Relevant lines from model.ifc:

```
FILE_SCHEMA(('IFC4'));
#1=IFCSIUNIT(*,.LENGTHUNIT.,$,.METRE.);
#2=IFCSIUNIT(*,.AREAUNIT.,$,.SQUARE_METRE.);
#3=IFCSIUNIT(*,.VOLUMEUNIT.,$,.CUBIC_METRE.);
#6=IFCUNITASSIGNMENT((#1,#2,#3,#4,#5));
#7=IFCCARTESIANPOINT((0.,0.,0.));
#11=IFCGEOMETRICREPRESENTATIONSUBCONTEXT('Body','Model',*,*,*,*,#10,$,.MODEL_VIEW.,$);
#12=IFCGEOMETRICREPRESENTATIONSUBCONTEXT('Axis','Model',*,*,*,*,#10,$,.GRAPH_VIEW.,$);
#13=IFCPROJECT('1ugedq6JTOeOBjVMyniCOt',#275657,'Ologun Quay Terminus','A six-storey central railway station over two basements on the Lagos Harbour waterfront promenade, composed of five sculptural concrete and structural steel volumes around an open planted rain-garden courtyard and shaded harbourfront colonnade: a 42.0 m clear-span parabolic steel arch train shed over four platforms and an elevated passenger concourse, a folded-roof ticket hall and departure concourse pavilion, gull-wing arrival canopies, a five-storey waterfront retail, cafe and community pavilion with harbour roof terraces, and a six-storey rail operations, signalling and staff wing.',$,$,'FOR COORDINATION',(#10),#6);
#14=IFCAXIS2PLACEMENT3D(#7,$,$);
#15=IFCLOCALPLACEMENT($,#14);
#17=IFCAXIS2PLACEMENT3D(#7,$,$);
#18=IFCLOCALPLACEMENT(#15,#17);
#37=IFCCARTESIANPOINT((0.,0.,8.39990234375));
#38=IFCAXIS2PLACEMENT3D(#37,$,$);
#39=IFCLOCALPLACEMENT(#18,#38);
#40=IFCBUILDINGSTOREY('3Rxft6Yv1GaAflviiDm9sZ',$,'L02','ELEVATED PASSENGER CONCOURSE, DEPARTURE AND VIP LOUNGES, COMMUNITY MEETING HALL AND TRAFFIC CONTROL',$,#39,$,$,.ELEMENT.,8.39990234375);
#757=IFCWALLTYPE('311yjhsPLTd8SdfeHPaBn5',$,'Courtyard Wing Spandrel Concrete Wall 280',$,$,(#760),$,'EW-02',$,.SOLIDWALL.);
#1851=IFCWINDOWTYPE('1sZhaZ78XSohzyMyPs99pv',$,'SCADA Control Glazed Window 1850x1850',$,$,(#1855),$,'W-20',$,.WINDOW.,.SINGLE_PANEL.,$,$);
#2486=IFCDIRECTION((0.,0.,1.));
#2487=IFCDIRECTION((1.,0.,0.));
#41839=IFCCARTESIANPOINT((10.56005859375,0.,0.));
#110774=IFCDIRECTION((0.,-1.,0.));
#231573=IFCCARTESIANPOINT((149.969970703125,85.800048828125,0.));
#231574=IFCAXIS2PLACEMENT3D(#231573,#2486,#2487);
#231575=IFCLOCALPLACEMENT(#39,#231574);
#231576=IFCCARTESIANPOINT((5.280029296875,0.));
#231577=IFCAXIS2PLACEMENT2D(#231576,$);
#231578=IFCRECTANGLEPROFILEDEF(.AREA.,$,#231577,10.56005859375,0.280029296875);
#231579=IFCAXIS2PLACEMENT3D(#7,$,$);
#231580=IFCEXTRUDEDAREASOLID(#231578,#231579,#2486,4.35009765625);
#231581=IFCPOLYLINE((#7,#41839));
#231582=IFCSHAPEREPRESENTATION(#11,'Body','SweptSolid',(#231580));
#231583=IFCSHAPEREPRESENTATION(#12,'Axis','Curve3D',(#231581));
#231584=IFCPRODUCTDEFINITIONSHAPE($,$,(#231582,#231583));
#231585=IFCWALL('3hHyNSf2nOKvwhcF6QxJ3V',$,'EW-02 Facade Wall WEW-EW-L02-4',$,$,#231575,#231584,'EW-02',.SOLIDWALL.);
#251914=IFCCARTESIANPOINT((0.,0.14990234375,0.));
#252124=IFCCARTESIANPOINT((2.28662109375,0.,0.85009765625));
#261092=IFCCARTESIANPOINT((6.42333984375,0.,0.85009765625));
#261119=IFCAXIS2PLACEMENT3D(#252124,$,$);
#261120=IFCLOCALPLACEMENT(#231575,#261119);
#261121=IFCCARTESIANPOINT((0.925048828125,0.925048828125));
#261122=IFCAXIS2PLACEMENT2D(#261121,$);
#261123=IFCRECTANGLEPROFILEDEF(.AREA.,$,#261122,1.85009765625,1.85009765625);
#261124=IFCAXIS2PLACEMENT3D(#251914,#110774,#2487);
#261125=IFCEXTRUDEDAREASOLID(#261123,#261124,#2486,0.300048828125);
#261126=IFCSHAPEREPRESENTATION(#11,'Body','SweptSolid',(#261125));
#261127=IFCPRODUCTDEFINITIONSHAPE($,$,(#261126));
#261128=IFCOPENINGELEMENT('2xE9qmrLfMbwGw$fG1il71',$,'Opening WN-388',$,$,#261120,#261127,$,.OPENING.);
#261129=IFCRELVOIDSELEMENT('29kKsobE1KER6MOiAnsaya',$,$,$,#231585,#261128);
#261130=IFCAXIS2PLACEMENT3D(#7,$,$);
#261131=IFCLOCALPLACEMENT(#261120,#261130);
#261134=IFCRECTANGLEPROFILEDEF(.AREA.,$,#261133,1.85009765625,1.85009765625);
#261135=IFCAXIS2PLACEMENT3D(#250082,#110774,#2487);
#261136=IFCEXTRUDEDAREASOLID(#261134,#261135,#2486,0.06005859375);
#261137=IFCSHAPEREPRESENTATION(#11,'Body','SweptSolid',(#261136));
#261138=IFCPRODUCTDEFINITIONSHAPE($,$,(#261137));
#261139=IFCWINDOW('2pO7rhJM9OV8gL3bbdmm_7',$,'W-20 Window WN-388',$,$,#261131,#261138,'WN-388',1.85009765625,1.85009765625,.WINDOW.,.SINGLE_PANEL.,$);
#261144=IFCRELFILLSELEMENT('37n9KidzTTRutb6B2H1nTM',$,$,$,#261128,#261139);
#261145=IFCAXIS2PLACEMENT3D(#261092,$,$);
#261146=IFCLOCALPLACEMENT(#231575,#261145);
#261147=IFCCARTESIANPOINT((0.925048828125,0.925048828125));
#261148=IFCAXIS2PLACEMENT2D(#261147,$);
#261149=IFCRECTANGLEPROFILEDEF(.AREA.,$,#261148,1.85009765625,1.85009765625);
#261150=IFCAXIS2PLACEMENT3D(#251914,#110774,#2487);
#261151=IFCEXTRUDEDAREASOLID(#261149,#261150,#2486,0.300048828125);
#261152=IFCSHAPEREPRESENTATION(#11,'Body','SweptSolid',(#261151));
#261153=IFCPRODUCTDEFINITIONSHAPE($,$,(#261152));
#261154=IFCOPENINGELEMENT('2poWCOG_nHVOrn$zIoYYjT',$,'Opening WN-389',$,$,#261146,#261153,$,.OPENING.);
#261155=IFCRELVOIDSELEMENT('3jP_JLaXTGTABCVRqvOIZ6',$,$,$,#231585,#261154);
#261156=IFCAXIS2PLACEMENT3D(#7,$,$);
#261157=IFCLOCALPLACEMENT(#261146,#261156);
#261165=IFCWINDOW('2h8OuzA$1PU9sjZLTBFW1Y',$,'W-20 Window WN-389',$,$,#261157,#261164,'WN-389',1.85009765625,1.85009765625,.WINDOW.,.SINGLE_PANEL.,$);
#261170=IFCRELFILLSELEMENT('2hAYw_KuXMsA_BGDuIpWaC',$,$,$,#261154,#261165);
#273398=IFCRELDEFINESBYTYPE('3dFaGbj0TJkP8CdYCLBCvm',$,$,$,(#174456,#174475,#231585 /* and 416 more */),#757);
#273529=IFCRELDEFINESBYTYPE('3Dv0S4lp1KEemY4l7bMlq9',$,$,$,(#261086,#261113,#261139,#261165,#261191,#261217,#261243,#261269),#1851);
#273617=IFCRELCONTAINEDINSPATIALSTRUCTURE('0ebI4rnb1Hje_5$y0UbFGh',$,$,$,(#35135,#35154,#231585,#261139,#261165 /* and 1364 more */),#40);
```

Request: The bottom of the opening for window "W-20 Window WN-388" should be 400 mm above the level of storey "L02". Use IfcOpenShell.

```python
import numpy as np
import ifcopenshell
import ifcopenshell.api.geometry
import ifcopenshell.geom
import ifcopenshell.util.element
import ifcopenshell.util.placement
import ifcopenshell.util.shape
import ifcopenshell.util.unit

model = ifcopenshell.open("model.ifc")
unit_scale = ifcopenshell.util.unit.calculate_unit_scale(model)

window = model.by_guid("2pO7rhJM9OV8gL3bbdmm_7")
opening = window.FillsVoids[0].RelatingOpeningElement
storey = ifcopenshell.util.element.get_container(window, ifc_class="IfcBuildingStorey")
level = ifcopenshell.util.placement.get_local_placement(storey.ObjectPlacement)[2, 3]

# The opening's origin need not be at the sill, so measure its lowest point.
shape = ifcopenshell.geom.create_shape(ifcopenshell.geom.settings(), opening)
bottom = ifcopenshell.util.shape.get_shape_bottom_elevation(shape, shape.geometry) / unit_scale
dz = level + 0.4 - bottom

shift = np.array([0.0, 0.0, dz])
# The window is placed relative to its opening, so it follows when the opening moves.
matrix = ifcopenshell.util.placement.get_local_placement(opening.ObjectPlacement)
matrix[:3, 3] += shift
ifcopenshell.api.geometry.edit_object_placement(
    model, product=opening, matrix=matrix, is_si=False, should_transform_children=True
)

print(f"moved by {dz * unit_scale:+.3f} m")

model.write("model_rev.ifc")
```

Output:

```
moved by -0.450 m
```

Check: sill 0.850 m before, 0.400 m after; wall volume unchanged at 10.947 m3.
